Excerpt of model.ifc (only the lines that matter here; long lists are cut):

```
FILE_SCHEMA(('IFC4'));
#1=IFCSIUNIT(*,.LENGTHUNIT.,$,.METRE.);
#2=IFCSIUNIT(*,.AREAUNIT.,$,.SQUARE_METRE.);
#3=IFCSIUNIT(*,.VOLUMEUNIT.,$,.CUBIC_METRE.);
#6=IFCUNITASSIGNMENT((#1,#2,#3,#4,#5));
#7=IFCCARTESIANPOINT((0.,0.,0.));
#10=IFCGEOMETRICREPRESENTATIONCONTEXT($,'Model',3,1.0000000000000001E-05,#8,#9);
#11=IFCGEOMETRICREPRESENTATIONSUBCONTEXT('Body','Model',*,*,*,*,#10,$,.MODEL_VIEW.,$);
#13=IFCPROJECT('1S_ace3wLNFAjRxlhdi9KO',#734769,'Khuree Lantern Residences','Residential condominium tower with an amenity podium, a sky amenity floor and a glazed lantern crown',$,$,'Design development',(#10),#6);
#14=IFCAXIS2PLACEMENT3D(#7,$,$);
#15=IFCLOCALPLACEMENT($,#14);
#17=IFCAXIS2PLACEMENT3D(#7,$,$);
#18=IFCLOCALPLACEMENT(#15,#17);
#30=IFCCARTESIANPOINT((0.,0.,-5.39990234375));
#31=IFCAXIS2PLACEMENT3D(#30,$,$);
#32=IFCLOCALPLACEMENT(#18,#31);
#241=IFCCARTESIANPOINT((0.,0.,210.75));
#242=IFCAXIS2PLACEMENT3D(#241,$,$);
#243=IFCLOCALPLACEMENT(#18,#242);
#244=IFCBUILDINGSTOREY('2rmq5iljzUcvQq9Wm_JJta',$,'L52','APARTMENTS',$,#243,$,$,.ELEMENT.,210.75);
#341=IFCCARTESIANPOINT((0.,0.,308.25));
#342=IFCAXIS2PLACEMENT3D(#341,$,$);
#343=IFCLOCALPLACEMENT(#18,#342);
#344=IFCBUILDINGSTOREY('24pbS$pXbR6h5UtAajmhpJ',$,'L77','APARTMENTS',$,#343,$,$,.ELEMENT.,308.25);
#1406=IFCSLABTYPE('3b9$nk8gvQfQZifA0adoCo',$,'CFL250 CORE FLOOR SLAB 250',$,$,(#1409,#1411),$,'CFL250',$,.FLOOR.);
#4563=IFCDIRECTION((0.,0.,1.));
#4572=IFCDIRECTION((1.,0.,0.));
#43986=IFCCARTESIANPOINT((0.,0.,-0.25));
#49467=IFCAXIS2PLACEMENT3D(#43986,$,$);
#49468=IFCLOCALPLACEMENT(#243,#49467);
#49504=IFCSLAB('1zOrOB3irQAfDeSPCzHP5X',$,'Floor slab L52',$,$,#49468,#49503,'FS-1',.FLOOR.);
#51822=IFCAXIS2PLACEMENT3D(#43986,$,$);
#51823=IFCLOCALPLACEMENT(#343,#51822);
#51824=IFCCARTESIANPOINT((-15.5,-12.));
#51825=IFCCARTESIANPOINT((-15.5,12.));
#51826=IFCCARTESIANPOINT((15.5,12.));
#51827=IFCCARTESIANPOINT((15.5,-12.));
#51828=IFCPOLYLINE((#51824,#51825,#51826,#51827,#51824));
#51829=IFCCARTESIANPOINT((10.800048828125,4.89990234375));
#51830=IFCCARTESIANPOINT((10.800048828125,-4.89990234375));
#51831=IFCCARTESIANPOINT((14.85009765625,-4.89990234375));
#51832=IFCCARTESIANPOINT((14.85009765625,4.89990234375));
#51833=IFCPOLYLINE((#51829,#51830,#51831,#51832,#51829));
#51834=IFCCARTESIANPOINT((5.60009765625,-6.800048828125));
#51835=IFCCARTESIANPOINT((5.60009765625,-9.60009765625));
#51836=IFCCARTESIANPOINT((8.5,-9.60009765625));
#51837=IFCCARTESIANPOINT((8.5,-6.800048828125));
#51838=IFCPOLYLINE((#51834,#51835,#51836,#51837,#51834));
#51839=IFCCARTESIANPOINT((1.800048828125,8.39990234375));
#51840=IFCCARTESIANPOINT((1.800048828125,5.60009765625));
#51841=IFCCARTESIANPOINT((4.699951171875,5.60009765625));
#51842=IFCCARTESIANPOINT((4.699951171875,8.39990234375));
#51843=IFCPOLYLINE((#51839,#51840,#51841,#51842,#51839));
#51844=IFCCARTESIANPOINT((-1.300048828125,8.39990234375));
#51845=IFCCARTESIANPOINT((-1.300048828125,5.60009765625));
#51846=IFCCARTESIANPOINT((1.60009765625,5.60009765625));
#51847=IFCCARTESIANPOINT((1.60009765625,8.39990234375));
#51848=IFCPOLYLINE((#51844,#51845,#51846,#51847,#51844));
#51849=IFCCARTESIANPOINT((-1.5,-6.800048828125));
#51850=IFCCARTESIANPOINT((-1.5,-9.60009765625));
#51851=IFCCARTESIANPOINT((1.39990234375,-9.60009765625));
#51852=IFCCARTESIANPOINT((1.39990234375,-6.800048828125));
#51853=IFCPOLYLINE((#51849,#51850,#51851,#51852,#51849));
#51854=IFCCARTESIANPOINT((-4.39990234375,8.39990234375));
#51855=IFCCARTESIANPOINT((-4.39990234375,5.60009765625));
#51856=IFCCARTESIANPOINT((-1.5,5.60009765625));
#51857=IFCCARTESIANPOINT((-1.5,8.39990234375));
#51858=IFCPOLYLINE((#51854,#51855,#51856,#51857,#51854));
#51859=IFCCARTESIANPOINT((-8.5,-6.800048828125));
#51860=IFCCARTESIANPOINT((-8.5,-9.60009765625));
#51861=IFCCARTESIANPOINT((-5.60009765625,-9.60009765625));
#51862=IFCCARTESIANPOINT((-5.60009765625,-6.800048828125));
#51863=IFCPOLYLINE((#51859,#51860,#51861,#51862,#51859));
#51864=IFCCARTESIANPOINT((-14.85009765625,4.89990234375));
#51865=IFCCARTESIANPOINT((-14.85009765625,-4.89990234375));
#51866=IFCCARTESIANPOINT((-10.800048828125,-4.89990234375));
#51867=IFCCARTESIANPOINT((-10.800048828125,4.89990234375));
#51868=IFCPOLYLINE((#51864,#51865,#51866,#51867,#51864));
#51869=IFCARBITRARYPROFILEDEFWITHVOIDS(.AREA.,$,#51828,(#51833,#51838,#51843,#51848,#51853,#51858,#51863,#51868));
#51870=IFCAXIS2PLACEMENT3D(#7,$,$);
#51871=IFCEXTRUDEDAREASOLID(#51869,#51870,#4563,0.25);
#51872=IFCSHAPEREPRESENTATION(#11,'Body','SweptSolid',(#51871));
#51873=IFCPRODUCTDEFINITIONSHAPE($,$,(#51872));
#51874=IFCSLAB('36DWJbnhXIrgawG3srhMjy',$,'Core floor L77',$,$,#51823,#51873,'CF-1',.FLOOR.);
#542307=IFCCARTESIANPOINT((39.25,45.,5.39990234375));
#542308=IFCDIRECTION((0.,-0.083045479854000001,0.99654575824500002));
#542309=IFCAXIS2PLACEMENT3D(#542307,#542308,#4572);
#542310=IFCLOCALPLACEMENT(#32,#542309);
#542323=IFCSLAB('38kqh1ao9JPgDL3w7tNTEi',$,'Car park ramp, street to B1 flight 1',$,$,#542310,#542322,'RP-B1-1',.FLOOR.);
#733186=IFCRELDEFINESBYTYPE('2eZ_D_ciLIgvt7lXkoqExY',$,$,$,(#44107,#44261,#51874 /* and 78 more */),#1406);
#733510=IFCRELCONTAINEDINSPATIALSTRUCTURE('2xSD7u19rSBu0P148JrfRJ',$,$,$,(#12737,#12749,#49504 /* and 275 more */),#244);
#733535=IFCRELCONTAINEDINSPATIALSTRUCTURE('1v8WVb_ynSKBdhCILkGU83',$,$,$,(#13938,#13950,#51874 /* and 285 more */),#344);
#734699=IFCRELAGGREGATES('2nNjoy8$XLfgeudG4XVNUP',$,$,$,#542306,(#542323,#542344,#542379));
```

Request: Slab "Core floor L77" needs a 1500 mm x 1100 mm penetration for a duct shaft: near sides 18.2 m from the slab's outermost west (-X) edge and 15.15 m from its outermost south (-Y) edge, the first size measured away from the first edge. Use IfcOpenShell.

```python
import numpy as np
import ifcopenshell
import ifcopenshell.api.feature
import ifcopenshell.api.geometry
import ifcopenshell.api.root
import ifcopenshell.geom
import ifcopenshell.util.placement
import ifcopenshell.util.representation
import ifcopenshell.util.shape
import ifcopenshell.util.unit

model = ifcopenshell.open("model.ifc")
unit_scale = ifcopenshell.util.unit.calculate_unit_scale(model)
settings = ifcopenshell.geom.settings()


def volume(element):
    """Net volume in cubic metres, openings subtracted."""
    shape = ifcopenshell.geom.create_shape(settings, element)
    return ifcopenshell.util.shape.get_volume(shape.geometry)


slab = model.by_guid("36DWJbnhXIrgawG3srhMjy")
before = volume(slab)

# Extent in the slab's own axes, in metres. The edges named are its -X and -Y sides.
slab_shape = ifcopenshell.geom.create_shape(settings, slab)
vertices = ifcopenshell.util.shape.get_vertices(slab_shape.geometry)
x_min, y_min, bottom = vertices.min(axis=0)
top = vertices[:, 2].max()

opening = ifcopenshell.api.root.create_entity(model, ifc_class="IfcOpeningElement", name="Duct shaft opening", predefined_type="OPENING")
context = ifcopenshell.util.representation.get_context(model, "Model", "Body", "MODEL_VIEW")
width, depth = 1.5, 1.1
outline = [(0.0, 0.0), (width, 0.0), (width, depth), (0.0, depth), (0.0, 0.0)]
# Overshoot both faces by 50 mm so the cut is clean.
shape = ifcopenshell.api.geometry.add_slab_representation(
    model, context=context, depth=top - bottom + 0.1, polyline=outline
)
ifcopenshell.api.geometry.assign_representation(model, product=opening, representation=shape)

matrix = ifcopenshell.util.placement.get_local_placement(slab.ObjectPlacement)
matrix[:, 3] = matrix @ np.append(np.array([x_min + 18.2, y_min + 15.15, bottom - 0.05]) / unit_scale, 1.0)
ifcopenshell.api.geometry.edit_object_placement(model, product=opening, matrix=matrix, is_si=False)
ifcopenshell.api.feature.add_feature(model, feature=opening, element=slab)

after = volume(slab)

print(f"slab volume {before:.3f} -> {after:.3f} m3")

model.write("model_updated.ifc")
```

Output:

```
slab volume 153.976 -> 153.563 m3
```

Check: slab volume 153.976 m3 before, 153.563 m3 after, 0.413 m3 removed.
